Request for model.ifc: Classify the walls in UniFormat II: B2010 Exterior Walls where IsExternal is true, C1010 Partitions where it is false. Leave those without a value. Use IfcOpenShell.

First a look at what the model holds.

```python
import ifcopenshell
import ifcopenshell.util.element

model = ifcopenshell.open("model.ifc")
print(model.schema)
print("classifications:", [c.Name for c in model.by_type("IfcClassification")])
values = [ifcopenshell.util.element.get_pset(e, "Pset_WallCommon", "IsExternal") for e in model.by_type("IfcWall")]
for value in (True, False, None):
    print("IsExternal", value, values.count(value))
```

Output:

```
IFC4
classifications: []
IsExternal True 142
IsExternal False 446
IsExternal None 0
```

```python
import ifcopenshell
import ifcopenshell.api.classification
import ifcopenshell.util.element

model = ifcopenshell.open("model.ifc")

system = ifcopenshell.api.classification.add_classification(model, classification="UniFormat II")

walls = model.by_type("IfcWall")
external = {e: ifcopenshell.util.element.get_pset(e, "Pset_WallCommon", "IsExternal") for e in walls}
for flag, code, name in ((True, "B2010", "Exterior Walls"), (False, "C1010", "Partitions")):
    products = [e for e in walls if external[e] is flag]
    ifcopenshell.api.classification.add_reference(
        model, products=products, classification=system, identification=code, name=name
    )
    print(code, len(products))

model.write("model-out.ifc")
```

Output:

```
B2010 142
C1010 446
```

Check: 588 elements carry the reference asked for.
